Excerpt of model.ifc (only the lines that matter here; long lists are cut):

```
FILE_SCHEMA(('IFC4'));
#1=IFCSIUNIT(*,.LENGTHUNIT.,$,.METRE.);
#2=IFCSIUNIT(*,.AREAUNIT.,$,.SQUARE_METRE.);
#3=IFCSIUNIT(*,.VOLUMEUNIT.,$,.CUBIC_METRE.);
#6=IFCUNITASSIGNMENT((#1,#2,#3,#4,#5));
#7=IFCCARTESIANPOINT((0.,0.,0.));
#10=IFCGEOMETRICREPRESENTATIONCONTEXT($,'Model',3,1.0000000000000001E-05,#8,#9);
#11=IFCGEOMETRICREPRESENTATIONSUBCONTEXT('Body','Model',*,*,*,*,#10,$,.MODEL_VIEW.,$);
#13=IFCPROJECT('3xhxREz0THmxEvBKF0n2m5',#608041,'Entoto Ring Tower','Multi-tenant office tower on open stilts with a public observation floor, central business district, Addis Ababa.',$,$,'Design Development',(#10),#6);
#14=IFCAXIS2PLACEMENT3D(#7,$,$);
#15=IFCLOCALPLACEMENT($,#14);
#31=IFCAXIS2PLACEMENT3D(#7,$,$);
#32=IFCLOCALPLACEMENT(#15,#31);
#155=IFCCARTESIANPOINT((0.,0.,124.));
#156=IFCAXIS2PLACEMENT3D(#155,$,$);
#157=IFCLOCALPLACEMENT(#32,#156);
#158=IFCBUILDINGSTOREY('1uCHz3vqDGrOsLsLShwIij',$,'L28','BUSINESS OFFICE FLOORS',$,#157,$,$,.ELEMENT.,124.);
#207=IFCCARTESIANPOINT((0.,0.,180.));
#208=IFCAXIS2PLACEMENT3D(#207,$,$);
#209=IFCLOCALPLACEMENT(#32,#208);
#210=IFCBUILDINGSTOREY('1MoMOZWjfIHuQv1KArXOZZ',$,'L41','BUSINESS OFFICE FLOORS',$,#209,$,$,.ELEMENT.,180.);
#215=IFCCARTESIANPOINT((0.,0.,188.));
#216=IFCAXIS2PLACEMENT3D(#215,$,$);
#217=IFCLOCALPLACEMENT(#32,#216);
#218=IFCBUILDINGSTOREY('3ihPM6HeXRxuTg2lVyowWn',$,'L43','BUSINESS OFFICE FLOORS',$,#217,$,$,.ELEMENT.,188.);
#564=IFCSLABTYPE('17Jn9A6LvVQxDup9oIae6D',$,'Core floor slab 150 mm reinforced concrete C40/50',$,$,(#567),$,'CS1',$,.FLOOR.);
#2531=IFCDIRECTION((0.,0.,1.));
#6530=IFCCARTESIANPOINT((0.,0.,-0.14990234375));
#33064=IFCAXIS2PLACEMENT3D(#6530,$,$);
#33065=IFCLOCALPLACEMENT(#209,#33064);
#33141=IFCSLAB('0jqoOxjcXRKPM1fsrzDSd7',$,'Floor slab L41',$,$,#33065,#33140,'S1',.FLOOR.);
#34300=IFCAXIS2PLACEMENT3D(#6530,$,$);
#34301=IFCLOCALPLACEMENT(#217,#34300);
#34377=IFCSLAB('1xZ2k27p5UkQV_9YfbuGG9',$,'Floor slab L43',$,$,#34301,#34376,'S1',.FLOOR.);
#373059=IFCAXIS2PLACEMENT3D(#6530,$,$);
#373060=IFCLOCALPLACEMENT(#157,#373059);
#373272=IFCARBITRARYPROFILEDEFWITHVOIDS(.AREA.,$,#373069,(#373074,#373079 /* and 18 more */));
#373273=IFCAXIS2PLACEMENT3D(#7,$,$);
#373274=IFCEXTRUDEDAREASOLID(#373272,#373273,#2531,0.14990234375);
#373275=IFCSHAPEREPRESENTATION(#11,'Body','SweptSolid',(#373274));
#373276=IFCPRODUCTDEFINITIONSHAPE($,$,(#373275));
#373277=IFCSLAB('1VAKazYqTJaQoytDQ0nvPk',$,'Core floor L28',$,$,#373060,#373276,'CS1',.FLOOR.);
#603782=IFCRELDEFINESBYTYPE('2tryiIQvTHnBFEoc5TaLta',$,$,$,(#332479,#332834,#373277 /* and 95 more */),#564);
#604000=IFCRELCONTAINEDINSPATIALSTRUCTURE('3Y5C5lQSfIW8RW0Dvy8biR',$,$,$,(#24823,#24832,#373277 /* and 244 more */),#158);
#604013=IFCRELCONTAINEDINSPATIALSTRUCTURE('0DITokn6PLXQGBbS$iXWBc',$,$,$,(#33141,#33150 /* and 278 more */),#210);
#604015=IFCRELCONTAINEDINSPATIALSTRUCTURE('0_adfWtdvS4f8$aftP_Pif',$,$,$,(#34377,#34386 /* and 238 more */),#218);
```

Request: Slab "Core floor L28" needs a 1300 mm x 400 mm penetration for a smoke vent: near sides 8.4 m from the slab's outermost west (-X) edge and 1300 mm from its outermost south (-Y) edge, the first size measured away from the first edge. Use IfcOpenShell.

```python
import numpy as np
import ifcopenshell
import ifcopenshell.api.feature
import ifcopenshell.api.geometry
import ifcopenshell.api.root
import ifcopenshell.geom
import ifcopenshell.util.placement
import ifcopenshell.util.representation
import ifcopenshell.util.shape
import ifcopenshell.util.unit

model = ifcopenshell.open("model.ifc")
unit_scale = ifcopenshell.util.unit.calculate_unit_scale(model)
settings = ifcopenshell.geom.settings()


def volume(element):
    """Net volume in cubic metres, openings subtracted."""
    shape = ifcopenshell.geom.create_shape(settings, element)
    return ifcopenshell.util.shape.get_volume(shape.geometry)


slab = model.by_guid("1VAKazYqTJaQoytDQ0nvPk")
before = volume(slab)

# Extent in the slab's own axes, in metres. The edges named are its -X and -Y sides.
slab_shape = ifcopenshell.geom.create_shape(settings, slab)
vertices = ifcopenshell.util.shape.get_vertices(slab_shape.geometry)
x_min, y_min, bottom = vertices.min(axis=0)
top = vertices[:, 2].max()

opening = ifcopenshell.api.root.create_entity(model, ifc_class="IfcOpeningElement", name="Smoke vent opening", predefined_type="OPENING")
context = ifcopenshell.util.representation.get_context(model, "Model", "Body", "MODEL_VIEW")
width, depth = 1.3, 0.4
outline = [(0.0, 0.0), (width, 0.0), (width, depth), (0.0, depth), (0.0, 0.0)]
# Overshoot both faces by 50 mm so the cut is clean.
shape = ifcopenshell.api.geometry.add_slab_representation(
    model, context=context, depth=top - bottom + 0.1, polyline=outline
)
ifcopenshell.api.geometry.assign_representation(model, product=opening, representation=shape)

matrix = ifcopenshell.util.placement.get_local_placement(slab.ObjectPlacement)
matrix[:, 3] = matrix @ np.append(np.array([x_min + 8.4, y_min + 1.3, bottom - 0.05]) / unit_scale, 1.0)
ifcopenshell.api.geometry.edit_object_placement(model, product=opening, matrix=matrix, is_si=False)
ifcopenshell.api.feature.add_feature(model, feature=opening, element=slab)

after = volume(slab)

print(f"slab volume {before:.3f} -> {after:.3f} m3")

model.write("model_v2.ifc")
```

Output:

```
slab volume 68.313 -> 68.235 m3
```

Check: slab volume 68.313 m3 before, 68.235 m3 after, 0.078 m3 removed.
